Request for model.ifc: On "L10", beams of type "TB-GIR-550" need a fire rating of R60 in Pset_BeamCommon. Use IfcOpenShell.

First a look at what the model holds.

```python
import ifcopenshell
import ifcopenshell.util.element

model = ifcopenshell.open("model.ifc")
print(model.schema)
storey = next(s for s in model.by_type("IfcBuildingStorey") if s.Name == "L10")
beams = [e for e in ifcopenshell.util.element.get_decomposition(storey) if e.is_a("IfcBeam")]
seen = {}
for e in beams:
    element_type = ifcopenshell.util.element.get_type(e)
    key = (element_type.Name if element_type != e and element_type else None, ifcopenshell.util.element.get_pset(e, "Pset_BeamCommon", "FireRating"))
    seen[key] = seen.get(key, 0) + 1
for (name, value), count in sorted(seen.items(), key=str):
    print(count, "x", name, "|", value)
```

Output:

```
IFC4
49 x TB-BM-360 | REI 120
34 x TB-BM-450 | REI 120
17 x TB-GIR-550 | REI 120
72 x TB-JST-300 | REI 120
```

```python
import ifcopenshell
import ifcopenshell.api.pset
import ifcopenshell.util.element

model = ifcopenshell.open("model.ifc")

storey = next(s for s in model.by_type("IfcBuildingStorey") if s.Name == "L10")
beams = [e for e in ifcopenshell.util.element.get_decomposition(storey) if e.is_a("IfcBeam")]

count = 0
for e in beams:
    element_type = ifcopenshell.util.element.get_type(e)
    if element_type in (None, e) or element_type.Name != "TB-GIR-550":
        continue
    # add_pset returns the element's existing set when there is one.
    pset = ifcopenshell.api.pset.add_pset(model, product=e, name="Pset_BeamCommon")
    ifcopenshell.api.pset.edit_pset(model, pset=pset, properties={"FireRating": "R60"})
    count += 1

print(count, "beams updated")

model.write("model_edited.ifc")
```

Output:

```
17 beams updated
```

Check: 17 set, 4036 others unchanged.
